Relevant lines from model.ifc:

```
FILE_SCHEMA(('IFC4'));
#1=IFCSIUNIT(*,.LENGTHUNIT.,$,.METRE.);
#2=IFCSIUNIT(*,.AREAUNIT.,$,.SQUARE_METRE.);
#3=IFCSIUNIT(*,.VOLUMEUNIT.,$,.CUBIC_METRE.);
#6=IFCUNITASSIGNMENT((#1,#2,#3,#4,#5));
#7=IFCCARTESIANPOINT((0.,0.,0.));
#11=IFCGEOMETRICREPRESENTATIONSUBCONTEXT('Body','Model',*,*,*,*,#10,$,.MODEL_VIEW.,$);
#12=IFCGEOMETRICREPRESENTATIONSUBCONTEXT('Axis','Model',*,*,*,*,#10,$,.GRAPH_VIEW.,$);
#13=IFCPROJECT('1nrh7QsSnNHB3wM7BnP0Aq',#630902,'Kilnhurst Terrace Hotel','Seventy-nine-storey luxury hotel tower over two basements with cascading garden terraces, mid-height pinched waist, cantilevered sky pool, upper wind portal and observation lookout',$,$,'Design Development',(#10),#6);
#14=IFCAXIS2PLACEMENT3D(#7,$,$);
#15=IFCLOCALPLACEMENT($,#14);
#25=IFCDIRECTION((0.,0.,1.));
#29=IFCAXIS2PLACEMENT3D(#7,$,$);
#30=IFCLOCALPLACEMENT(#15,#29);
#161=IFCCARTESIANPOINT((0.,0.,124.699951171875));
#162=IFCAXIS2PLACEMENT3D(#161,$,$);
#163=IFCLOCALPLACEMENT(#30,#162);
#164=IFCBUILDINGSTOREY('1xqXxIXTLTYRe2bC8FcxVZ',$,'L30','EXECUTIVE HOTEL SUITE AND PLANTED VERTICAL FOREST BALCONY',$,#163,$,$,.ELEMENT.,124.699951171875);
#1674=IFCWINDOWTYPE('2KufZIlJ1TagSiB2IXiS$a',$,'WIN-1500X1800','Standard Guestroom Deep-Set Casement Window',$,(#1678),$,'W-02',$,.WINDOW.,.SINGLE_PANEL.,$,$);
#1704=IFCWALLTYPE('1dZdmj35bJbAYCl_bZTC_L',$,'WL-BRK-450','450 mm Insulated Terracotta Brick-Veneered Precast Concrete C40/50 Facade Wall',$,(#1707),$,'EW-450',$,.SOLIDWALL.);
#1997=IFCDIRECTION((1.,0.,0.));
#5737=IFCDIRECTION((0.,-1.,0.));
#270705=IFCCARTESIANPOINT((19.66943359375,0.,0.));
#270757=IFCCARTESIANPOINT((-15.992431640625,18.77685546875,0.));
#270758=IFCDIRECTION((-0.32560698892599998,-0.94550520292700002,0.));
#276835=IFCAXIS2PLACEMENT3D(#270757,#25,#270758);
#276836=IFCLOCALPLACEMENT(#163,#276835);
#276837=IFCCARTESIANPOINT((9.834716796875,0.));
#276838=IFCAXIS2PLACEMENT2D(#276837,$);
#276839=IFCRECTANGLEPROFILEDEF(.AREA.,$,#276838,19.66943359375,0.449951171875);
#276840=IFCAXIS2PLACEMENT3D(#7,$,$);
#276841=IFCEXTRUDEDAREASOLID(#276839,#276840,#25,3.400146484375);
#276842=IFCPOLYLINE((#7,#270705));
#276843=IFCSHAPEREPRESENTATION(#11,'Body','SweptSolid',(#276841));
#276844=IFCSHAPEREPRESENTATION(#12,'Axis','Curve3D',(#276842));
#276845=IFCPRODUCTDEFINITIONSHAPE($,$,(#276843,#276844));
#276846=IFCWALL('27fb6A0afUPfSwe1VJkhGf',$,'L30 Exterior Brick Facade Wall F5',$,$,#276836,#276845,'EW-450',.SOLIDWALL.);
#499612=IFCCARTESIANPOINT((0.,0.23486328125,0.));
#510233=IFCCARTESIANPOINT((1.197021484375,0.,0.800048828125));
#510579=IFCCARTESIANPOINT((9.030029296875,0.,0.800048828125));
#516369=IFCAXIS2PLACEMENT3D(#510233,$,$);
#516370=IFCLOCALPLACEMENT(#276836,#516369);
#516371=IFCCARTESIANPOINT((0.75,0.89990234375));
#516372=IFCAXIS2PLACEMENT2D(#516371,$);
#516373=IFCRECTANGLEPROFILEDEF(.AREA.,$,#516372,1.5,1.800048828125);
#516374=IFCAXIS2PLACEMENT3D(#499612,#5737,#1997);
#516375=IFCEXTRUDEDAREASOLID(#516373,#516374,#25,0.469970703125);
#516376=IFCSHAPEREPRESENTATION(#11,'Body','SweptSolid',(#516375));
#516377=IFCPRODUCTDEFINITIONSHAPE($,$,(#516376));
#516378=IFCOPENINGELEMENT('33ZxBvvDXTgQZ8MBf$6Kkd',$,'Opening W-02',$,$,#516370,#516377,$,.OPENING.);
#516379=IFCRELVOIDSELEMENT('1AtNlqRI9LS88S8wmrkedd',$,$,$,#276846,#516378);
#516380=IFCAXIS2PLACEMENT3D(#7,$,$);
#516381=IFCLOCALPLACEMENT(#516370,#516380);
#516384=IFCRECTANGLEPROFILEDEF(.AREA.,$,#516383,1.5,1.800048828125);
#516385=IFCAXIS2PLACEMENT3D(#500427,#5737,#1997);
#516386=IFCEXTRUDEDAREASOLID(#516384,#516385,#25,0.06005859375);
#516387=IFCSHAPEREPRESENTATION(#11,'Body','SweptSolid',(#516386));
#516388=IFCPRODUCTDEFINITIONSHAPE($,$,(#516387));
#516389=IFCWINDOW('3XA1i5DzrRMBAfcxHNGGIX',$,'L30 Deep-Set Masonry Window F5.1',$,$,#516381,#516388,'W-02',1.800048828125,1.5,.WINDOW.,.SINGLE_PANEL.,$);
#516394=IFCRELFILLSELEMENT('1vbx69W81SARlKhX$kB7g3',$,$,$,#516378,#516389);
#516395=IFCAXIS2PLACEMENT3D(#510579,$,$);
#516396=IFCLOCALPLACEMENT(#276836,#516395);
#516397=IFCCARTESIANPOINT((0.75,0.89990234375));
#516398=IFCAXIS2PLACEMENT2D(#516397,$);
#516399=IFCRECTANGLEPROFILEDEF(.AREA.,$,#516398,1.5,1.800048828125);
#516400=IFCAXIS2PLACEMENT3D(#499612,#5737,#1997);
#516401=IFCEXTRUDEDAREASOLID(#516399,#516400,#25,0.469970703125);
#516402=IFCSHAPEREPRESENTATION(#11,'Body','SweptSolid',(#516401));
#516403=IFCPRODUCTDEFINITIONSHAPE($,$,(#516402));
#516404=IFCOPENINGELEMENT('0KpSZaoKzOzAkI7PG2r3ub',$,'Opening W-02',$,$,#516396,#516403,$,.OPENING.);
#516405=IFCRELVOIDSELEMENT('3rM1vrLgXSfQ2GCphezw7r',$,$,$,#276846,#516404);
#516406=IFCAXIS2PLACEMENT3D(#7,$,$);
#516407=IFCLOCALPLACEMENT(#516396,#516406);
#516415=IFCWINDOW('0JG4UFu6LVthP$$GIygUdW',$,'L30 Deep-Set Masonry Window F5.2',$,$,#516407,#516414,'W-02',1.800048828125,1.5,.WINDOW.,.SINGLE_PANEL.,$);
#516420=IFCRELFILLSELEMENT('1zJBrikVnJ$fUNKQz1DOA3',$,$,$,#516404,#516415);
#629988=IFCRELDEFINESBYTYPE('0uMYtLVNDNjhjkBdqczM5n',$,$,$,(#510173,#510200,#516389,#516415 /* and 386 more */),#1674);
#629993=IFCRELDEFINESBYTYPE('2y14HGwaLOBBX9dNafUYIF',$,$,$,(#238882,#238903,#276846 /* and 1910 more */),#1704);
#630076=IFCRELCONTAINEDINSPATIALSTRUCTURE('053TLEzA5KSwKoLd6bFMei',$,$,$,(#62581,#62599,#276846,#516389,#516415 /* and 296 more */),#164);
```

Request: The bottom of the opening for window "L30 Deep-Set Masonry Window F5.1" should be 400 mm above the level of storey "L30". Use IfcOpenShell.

```python
import numpy as np
import ifcopenshell
import ifcopenshell.api.geometry
import ifcopenshell.geom
import ifcopenshell.util.element
import ifcopenshell.util.placement
import ifcopenshell.util.shape
import ifcopenshell.util.unit

model = ifcopenshell.open("model.ifc")
unit_scale = ifcopenshell.util.unit.calculate_unit_scale(model)

window = model.by_guid("3XA1i5DzrRMBAfcxHNGGIX")
opening = window.FillsVoids[0].RelatingOpeningElement
storey = ifcopenshell.util.element.get_container(window, ifc_class="IfcBuildingStorey")
level = ifcopenshell.util.placement.get_local_placement(storey.ObjectPlacement)[2, 3]

# The opening's origin need not be at the sill, so measure its lowest point.
shape = ifcopenshell.geom.create_shape(ifcopenshell.geom.settings(), opening)
bottom = ifcopenshell.util.shape.get_shape_bottom_elevation(shape, shape.geometry) / unit_scale
dz = level + 0.4 - bottom

shift = np.array([0.0, 0.0, dz])
# The window is placed relative to its opening, so it follows when the opening moves.
matrix = ifcopenshell.util.placement.get_local_placement(opening.ObjectPlacement)
matrix[:3, 3] += shift
ifcopenshell.api.geometry.edit_object_placement(
    model, product=opening, matrix=matrix, is_si=False, should_transform_children=True
)

print(f"moved by {dz * unit_scale:+.3f} m")

model.write("model_rev.ifc")
```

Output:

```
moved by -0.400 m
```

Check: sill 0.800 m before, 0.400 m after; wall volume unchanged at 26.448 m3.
